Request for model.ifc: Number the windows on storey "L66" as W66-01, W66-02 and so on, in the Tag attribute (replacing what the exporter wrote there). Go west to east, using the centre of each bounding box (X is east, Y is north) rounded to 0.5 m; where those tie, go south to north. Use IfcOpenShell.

First a look at what the model holds.

```python
import ifcopenshell
import ifcopenshell.util.element
import ifcopenshell.util.placement

model = ifcopenshell.open("model.ifc")
print(model.schema)
storey = next(s for s in model.by_type("IfcBuildingStorey") if s.Name == "L66")
windows = [e for e in ifcopenshell.util.element.get_decomposition(storey) if e.is_a("IfcWindow")]
for e in sorted(windows, key=lambda e: e.id()):
    origin = ifcopenshell.util.placement.get_local_placement(e.ObjectPlacement)[:3, 3]
    print(e.id(), e.Tag, e.Name, origin.round(2) + 0.0, sep=" | ")
```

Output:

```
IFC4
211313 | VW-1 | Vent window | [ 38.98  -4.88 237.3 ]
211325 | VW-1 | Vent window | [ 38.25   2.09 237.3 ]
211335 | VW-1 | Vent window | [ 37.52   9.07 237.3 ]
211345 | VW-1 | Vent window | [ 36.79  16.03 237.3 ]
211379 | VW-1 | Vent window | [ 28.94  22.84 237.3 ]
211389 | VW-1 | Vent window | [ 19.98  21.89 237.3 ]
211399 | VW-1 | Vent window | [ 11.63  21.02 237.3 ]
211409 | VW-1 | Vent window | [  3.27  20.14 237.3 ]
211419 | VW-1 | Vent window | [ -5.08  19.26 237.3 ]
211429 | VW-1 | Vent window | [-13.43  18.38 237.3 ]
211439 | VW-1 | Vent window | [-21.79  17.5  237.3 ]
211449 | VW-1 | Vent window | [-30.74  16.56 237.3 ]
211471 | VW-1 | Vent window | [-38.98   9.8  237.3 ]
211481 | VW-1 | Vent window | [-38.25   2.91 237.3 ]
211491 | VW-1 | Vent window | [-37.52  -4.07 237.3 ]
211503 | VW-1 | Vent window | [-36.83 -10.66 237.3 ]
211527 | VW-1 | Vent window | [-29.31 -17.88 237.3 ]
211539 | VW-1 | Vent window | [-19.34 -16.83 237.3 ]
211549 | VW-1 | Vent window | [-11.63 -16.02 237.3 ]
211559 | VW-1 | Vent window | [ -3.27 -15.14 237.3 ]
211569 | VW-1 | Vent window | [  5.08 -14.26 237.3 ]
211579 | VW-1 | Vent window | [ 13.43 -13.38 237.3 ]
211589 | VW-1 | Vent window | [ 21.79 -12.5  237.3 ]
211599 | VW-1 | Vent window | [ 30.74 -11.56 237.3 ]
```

```python
import ifcopenshell
import ifcopenshell.geom
import ifcopenshell.util.element
import ifcopenshell.util.shape

model = ifcopenshell.open("model.ifc")
settings = ifcopenshell.geom.settings()
settings.set("use-world-coords", True)


def centre(element):
    shape = ifcopenshell.geom.create_shape(settings, element)
    return ifcopenshell.util.shape.get_bbox_centroid(shape.geometry)


storey = next(s for s in model.by_type("IfcBuildingStorey") if s.Name == "L66")
windows = [e for e in ifcopenshell.util.element.get_decomposition(storey) if e.is_a("IfcWindow")]

# Insertion points can sit at a corner or the storey origin, so sort by the geometry (in metres).
centres = {e: centre(e) for e in windows}
windows.sort(key=lambda e: (round(centres[e][0] / 0.5), centres[e][1]))

for i, e in enumerate(windows, start=1):
    number = f"W66-{i:02d}"
    e.Tag = number
    print(e.id(), number)

model.write("model_rev.ifc")
```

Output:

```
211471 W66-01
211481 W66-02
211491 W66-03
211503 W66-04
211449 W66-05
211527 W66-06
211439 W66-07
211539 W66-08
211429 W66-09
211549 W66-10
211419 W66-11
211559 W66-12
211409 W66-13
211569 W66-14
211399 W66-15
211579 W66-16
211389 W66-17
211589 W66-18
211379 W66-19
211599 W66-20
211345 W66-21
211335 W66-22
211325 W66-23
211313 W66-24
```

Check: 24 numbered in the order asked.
